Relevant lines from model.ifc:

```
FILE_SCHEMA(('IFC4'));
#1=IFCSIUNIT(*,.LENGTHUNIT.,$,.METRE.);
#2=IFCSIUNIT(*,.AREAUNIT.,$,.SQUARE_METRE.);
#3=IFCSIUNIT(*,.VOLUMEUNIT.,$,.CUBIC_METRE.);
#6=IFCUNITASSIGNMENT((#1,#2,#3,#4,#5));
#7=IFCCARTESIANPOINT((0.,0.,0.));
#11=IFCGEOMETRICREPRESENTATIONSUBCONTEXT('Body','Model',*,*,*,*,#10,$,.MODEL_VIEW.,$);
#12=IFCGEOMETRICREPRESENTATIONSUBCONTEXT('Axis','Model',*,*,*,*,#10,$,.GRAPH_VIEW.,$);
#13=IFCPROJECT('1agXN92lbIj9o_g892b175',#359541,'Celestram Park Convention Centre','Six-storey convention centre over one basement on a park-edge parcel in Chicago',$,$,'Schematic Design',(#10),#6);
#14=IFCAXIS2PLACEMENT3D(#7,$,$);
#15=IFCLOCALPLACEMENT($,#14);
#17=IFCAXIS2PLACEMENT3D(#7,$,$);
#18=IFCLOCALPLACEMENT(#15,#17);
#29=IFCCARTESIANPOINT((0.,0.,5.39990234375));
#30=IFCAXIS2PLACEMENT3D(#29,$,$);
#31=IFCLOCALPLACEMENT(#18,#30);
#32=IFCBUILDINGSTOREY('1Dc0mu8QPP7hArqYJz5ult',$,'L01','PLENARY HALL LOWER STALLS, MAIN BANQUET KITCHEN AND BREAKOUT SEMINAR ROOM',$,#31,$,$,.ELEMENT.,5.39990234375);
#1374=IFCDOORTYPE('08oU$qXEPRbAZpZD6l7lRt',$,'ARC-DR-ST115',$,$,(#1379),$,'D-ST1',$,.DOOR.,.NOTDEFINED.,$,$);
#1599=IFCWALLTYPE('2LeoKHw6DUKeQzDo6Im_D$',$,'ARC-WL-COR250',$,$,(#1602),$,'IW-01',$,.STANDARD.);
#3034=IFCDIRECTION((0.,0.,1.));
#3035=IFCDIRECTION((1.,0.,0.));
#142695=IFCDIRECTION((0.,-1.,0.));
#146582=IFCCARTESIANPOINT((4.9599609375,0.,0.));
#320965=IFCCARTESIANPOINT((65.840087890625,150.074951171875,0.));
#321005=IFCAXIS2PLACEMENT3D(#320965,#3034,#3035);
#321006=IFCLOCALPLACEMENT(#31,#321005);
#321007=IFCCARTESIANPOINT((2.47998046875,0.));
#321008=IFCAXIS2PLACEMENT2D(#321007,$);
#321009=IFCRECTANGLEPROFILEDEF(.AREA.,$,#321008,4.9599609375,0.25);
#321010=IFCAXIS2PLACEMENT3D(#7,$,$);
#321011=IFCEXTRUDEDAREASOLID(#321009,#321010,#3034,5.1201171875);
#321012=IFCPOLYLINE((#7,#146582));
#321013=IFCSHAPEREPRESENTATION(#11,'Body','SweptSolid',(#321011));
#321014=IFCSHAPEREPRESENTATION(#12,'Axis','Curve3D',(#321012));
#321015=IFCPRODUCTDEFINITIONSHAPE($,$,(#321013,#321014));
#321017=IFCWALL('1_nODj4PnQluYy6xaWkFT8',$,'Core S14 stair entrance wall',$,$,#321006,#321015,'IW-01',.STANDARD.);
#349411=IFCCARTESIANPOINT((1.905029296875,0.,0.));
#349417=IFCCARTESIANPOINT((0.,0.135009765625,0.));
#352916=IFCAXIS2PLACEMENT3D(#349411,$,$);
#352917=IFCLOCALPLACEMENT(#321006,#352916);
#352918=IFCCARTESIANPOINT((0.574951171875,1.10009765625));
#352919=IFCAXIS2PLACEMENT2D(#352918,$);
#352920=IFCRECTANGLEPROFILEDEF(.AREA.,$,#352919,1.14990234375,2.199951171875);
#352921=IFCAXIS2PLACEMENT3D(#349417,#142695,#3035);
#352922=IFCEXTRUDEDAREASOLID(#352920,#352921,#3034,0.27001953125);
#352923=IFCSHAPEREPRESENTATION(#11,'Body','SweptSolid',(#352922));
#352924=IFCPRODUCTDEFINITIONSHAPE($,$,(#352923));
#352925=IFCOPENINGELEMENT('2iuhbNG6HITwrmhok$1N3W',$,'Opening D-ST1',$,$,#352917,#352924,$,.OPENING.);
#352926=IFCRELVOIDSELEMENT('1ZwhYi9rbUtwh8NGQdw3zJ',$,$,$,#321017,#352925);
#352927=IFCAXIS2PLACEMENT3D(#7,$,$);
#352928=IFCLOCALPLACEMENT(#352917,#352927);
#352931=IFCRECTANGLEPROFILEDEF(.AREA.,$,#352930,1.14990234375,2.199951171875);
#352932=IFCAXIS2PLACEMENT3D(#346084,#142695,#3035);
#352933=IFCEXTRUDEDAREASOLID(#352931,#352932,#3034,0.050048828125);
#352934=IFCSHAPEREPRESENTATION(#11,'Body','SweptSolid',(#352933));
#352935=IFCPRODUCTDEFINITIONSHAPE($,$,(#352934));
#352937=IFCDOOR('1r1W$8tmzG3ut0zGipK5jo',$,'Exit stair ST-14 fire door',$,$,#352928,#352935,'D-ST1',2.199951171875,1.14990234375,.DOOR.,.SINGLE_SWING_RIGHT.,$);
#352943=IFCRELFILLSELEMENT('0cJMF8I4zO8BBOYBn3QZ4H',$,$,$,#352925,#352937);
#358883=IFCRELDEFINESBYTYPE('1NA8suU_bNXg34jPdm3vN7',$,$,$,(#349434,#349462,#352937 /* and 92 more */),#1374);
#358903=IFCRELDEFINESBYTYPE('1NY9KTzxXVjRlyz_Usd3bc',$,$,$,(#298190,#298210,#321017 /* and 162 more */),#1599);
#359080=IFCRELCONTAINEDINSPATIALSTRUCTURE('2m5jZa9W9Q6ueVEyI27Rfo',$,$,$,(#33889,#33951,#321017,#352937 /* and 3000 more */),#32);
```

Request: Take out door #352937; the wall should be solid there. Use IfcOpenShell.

```python
import ifcopenshell
import ifcopenshell.api.feature
import ifcopenshell.api.root
import ifcopenshell.geom
import ifcopenshell.util.shape

model = ifcopenshell.open("model.ifc")
settings = ifcopenshell.geom.settings()


def volume(element):
    """Net volume in cubic metres, openings subtracted."""
    shape = ifcopenshell.geom.create_shape(settings, element)
    return ifcopenshell.util.shape.get_volume(shape.geometry)


door = model.by_guid("1r1W$8tmzG3ut0zGipK5jo")
opening = door.FillsVoids[0].RelatingOpeningElement
wall = opening.VoidsElements[0].RelatingBuildingElement
before = volume(wall)

ifcopenshell.api.root.remove_product(model, product=door)
ifcopenshell.api.feature.remove_feature(model, feature=opening)

after = volume(wall)

print(f"wall volume {before:.3f} -> {after:.3f} m3")

model.write("model-out.ifc")
```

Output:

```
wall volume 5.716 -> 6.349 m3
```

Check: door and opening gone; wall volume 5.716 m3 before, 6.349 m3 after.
